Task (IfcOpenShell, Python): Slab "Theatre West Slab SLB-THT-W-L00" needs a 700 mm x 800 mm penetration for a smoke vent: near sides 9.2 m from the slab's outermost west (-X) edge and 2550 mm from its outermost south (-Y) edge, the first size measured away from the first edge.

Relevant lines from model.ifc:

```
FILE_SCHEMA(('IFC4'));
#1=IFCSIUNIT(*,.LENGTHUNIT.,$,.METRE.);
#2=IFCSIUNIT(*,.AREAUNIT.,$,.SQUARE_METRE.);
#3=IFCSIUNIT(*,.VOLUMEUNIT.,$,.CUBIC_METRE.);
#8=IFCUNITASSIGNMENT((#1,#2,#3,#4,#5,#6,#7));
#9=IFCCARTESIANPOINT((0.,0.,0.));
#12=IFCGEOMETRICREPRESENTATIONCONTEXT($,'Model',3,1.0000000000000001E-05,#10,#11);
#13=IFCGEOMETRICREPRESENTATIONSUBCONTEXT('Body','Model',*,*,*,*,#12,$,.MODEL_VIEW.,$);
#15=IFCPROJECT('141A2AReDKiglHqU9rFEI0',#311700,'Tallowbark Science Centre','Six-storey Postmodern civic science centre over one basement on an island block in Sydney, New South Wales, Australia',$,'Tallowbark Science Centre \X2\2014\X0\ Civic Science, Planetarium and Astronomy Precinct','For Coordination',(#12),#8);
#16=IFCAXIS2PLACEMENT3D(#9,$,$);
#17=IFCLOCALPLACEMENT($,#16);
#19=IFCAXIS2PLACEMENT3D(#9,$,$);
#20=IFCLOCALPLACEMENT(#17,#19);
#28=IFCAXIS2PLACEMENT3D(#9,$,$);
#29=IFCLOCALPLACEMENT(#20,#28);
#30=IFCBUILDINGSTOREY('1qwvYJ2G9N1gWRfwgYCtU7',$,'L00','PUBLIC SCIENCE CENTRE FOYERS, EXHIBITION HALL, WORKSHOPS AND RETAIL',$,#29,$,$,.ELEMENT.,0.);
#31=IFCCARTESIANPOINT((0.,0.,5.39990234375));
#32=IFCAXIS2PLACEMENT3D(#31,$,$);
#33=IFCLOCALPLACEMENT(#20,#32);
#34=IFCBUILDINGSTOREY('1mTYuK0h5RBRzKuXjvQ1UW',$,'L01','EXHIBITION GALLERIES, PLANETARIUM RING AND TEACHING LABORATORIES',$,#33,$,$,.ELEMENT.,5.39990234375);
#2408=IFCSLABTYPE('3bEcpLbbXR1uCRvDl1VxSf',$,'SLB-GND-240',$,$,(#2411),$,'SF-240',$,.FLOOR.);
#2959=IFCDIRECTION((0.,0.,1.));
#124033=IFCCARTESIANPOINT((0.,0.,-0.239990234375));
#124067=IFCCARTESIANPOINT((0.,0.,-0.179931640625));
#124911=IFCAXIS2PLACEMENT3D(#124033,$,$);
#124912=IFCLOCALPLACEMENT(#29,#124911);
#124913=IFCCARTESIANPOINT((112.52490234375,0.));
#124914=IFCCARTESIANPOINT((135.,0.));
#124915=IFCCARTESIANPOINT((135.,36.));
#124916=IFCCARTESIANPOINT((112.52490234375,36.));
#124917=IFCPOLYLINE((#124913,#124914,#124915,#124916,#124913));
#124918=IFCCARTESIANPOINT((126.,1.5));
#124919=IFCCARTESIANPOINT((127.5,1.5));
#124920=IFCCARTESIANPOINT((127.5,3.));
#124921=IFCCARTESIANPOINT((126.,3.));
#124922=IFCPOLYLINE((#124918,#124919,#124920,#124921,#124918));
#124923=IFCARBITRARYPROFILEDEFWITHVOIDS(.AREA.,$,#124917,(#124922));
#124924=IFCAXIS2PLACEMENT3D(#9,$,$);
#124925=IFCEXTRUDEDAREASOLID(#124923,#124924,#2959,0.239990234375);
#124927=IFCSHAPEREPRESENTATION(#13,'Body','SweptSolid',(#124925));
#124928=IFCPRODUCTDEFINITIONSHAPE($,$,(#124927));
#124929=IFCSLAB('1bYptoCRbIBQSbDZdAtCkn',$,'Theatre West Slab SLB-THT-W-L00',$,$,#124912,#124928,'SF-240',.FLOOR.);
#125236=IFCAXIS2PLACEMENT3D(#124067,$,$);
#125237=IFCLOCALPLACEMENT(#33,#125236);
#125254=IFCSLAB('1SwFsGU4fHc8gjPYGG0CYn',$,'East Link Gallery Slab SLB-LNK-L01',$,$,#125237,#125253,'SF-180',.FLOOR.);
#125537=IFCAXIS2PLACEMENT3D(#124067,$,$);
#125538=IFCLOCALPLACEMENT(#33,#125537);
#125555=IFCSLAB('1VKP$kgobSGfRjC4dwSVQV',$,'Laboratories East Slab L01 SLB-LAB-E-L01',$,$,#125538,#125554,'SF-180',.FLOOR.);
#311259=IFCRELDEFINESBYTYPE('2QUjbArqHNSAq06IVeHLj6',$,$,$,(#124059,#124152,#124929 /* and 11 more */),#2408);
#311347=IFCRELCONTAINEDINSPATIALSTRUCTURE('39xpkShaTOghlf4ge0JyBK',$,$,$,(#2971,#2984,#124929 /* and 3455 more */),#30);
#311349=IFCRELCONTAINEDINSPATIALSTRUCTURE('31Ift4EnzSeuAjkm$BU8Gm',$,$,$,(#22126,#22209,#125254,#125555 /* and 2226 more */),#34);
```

```python
import numpy as np
import ifcopenshell
import ifcopenshell.api.feature
import ifcopenshell.api.geometry
import ifcopenshell.api.root
import ifcopenshell.geom
import ifcopenshell.util.placement
import ifcopenshell.util.representation
import ifcopenshell.util.shape
import ifcopenshell.util.unit

model = ifcopenshell.open("model.ifc")
unit_scale = ifcopenshell.util.unit.calculate_unit_scale(model)
settings = ifcopenshell.geom.settings()


def volume(element):
    """Net volume in cubic metres, openings subtracted."""
    shape = ifcopenshell.geom.create_shape(settings, element)
    return ifcopenshell.util.shape.get_volume(shape.geometry)


slab = model.by_guid("1bYptoCRbIBQSbDZdAtCkn")
before = volume(slab)

# Extent in the slab's own axes, in metres. The edges named are its -X and -Y sides.
slab_shape = ifcopenshell.geom.create_shape(settings, slab)
vertices = ifcopenshell.util.shape.get_vertices(slab_shape.geometry)
x_min, y_min, bottom = vertices.min(axis=0)
top = vertices[:, 2].max()

opening = ifcopenshell.api.root.create_entity(model, ifc_class="IfcOpeningElement", name="Smoke vent opening", predefined_type="OPENING")
context = ifcopenshell.util.representation.get_context(model, "Model", "Body", "MODEL_VIEW")
width, depth = 0.7, 0.8
outline = [(0.0, 0.0), (width, 0.0), (width, depth), (0.0, depth), (0.0, 0.0)]
# Overshoot both faces by 50 mm so the cut is clean.
shape = ifcopenshell.api.geometry.add_slab_representation(
    model, context=context, depth=top - bottom + 0.1, polyline=outline
)
ifcopenshell.api.geometry.assign_representation(model, product=opening, representation=shape)

matrix = ifcopenshell.util.placement.get_local_placement(slab.ObjectPlacement)
matrix[:, 3] = matrix @ np.append(np.array([x_min + 9.2, y_min + 2.55, bottom - 0.05]) / unit_scale, 1.0)
ifcopenshell.api.geometry.edit_object_placement(model, product=opening, matrix=matrix, is_si=False)
ifcopenshell.api.feature.add_feature(model, feature=opening, element=slab)

after = volume(slab)

print(f"slab volume {before:.3f} -> {after:.3f} m3")

model.write("model_updated.ifc")
```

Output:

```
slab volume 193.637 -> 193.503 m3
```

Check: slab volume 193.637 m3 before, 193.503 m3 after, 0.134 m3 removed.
